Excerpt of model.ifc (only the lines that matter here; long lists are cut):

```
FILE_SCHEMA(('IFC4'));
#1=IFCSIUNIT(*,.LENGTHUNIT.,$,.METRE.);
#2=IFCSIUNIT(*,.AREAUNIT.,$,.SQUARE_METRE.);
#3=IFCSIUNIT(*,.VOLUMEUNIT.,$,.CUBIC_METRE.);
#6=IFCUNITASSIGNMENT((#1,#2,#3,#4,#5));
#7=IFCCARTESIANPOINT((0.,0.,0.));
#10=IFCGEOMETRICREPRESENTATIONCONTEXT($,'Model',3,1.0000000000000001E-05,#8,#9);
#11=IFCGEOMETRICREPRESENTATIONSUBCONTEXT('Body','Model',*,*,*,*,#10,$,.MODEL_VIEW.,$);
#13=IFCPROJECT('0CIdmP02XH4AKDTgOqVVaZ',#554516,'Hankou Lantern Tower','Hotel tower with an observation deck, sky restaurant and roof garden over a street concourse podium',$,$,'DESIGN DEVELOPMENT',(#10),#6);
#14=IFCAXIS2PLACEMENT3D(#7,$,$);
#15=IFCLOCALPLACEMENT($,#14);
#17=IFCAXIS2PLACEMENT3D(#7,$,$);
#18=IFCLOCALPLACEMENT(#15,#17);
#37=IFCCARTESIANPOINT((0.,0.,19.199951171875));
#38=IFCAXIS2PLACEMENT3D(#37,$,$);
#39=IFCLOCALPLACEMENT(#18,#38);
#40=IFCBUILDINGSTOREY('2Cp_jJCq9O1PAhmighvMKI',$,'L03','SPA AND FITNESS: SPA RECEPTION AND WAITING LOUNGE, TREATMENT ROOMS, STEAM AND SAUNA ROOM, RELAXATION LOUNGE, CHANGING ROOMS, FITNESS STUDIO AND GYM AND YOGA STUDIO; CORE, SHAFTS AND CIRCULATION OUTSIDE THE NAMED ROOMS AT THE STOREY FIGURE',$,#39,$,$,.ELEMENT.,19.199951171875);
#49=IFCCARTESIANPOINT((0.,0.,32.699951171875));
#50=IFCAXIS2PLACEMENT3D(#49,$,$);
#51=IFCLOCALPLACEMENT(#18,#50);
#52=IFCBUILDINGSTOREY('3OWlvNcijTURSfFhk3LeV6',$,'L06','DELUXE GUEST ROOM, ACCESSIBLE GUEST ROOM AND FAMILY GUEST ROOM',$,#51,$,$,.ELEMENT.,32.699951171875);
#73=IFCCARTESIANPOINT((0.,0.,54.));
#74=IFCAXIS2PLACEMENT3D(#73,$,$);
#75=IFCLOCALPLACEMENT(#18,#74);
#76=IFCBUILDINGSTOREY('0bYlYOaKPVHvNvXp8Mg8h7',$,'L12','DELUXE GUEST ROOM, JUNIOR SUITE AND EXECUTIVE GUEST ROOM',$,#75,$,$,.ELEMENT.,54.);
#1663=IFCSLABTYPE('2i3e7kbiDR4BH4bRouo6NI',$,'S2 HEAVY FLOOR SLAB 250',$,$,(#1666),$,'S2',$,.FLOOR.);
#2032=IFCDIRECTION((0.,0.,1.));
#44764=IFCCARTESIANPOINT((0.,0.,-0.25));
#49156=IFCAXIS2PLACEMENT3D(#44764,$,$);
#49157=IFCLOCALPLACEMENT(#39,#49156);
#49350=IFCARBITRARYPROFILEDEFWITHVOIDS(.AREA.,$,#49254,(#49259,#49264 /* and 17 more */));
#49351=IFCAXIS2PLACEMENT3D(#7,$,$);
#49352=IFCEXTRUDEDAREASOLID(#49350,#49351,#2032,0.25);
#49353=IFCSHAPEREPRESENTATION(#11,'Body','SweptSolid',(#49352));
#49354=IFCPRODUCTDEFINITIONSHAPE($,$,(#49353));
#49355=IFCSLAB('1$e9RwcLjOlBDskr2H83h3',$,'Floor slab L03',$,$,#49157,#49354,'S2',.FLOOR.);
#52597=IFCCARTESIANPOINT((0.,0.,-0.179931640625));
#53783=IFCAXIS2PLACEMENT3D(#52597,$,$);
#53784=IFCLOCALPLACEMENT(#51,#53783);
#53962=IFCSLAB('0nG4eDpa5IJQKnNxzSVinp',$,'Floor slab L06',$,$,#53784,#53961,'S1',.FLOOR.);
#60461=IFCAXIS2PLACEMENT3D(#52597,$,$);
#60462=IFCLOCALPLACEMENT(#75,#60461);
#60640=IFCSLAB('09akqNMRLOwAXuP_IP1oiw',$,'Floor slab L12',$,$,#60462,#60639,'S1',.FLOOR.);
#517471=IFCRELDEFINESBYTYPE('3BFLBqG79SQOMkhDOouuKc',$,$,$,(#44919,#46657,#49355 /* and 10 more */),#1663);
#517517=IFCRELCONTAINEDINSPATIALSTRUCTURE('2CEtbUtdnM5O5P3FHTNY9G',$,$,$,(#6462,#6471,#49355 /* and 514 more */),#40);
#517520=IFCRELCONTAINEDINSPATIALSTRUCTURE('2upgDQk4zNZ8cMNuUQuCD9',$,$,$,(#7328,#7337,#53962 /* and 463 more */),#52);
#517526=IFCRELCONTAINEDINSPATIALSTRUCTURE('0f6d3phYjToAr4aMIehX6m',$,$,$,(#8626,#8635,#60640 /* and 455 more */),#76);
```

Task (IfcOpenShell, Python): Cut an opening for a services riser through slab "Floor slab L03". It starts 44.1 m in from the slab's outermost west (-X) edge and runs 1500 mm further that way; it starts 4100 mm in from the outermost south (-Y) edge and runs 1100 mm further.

```python
import numpy as np
import ifcopenshell
import ifcopenshell.api.feature
import ifcopenshell.api.geometry
import ifcopenshell.api.root
import ifcopenshell.geom
import ifcopenshell.util.placement
import ifcopenshell.util.representation
import ifcopenshell.util.shape
import ifcopenshell.util.unit

model = ifcopenshell.open("model.ifc")
unit_scale = ifcopenshell.util.unit.calculate_unit_scale(model)
settings = ifcopenshell.geom.settings()


def volume(element):
    """Net volume in cubic metres, openings subtracted."""
    shape = ifcopenshell.geom.create_shape(settings, element)
    return ifcopenshell.util.shape.get_volume(shape.geometry)


slab = model.by_id(49355)
before = volume(slab)

# Extent in the slab's own axes, in metres. The edges named are its -X and -Y sides.
slab_shape = ifcopenshell.geom.create_shape(settings, slab)
vertices = ifcopenshell.util.shape.get_vertices(slab_shape.geometry)
x_min, y_min, bottom = vertices.min(axis=0)
top = vertices[:, 2].max()

opening = ifcopenshell.api.root.create_entity(model, ifc_class="IfcOpeningElement", name="Services riser opening", predefined_type="OPENING")
context = ifcopenshell.util.representation.get_context(model, "Model", "Body", "MODEL_VIEW")
width, depth = 1.5, 1.1
outline = [(0.0, 0.0), (width, 0.0), (width, depth), (0.0, depth), (0.0, 0.0)]
# Overshoot both faces by 50 mm so the cut is clean.
shape = ifcopenshell.api.geometry.add_slab_representation(
    model, context=context, depth=top - bottom + 0.1, polyline=outline
)
ifcopenshell.api.geometry.assign_representation(model, product=opening, representation=shape)

matrix = ifcopenshell.util.placement.get_local_placement(slab.ObjectPlacement)
matrix[:, 3] = matrix @ np.append(np.array([x_min + 44.1, y_min + 4.1, bottom - 0.05]) / unit_scale, 1.0)
ifcopenshell.api.geometry.edit_object_placement(model, product=opening, matrix=matrix, is_si=False)
ifcopenshell.api.feature.add_feature(model, feature=opening, element=slab)

after = volume(slab)

print(f"slab volume {before:.3f} -> {after:.3f} m3")

model.write("model-out.ifc")
```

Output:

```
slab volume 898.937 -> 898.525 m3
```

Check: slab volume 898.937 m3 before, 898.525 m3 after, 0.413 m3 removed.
